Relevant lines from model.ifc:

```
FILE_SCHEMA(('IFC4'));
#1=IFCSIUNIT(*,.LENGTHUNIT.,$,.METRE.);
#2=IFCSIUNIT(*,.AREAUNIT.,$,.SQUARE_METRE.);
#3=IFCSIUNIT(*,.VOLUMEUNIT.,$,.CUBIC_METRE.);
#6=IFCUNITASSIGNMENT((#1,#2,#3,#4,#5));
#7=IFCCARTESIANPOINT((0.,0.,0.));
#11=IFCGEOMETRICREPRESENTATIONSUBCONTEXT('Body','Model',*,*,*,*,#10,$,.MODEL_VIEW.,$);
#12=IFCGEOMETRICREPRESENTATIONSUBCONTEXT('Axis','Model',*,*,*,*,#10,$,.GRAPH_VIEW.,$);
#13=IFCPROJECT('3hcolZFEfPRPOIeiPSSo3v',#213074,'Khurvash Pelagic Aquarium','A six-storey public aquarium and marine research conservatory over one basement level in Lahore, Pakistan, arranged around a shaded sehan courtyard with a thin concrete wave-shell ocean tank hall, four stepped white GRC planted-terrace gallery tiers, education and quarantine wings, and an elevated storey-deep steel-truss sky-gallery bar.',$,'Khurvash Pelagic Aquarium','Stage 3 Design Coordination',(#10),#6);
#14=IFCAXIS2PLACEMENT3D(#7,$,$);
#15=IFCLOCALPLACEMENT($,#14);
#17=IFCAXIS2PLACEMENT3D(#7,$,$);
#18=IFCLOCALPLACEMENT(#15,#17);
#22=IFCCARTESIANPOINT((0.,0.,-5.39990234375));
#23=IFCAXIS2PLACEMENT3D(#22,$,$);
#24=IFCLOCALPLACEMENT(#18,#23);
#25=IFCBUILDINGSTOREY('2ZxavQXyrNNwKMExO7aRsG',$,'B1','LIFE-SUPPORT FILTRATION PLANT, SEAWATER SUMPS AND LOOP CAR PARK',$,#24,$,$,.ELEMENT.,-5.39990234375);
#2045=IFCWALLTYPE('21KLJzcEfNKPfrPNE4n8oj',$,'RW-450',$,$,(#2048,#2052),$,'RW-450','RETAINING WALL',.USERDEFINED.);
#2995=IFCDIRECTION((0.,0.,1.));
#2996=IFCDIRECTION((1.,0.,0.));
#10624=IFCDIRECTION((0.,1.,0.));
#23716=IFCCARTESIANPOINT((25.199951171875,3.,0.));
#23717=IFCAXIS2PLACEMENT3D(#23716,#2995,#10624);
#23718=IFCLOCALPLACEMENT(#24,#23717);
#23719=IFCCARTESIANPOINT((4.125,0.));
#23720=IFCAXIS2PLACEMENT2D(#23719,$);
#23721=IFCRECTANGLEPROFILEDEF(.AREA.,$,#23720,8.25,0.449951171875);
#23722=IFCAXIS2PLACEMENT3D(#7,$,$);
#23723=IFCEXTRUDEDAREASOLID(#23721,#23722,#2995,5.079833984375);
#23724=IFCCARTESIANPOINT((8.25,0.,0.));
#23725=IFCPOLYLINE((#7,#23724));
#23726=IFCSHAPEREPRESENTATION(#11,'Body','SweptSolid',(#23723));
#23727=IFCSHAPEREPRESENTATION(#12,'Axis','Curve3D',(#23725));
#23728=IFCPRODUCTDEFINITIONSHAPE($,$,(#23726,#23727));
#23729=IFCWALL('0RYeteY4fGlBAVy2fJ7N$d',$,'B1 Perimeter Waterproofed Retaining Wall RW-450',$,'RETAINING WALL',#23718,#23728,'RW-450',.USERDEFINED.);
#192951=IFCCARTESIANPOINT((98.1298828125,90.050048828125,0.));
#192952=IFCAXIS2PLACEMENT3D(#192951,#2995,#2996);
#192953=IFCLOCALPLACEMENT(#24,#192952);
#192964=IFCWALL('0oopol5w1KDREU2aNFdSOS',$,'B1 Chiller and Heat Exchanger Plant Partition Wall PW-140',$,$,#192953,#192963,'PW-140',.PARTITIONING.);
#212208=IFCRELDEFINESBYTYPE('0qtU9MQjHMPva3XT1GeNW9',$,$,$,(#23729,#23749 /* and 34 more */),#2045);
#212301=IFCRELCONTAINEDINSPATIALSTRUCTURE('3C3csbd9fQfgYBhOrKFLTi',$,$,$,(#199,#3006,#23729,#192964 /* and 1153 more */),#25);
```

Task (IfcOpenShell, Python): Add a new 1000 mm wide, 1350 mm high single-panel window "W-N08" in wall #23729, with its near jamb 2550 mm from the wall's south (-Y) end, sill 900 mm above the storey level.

```python
import numpy as np
import ifcopenshell
import ifcopenshell.api.feature
import ifcopenshell.api.geometry
import ifcopenshell.api.root
import ifcopenshell.api.spatial
import ifcopenshell.geom
import ifcopenshell.util.element
import ifcopenshell.util.placement
import ifcopenshell.util.representation
import ifcopenshell.util.shape
import ifcopenshell.util.unit

model = ifcopenshell.open("model.ifc")
unit_scale = ifcopenshell.util.unit.calculate_unit_scale(model)
settings = ifcopenshell.geom.settings()


def volume(element):
    """Net volume in cubic metres, openings subtracted."""
    shape = ifcopenshell.geom.create_shape(settings, element)
    return ifcopenshell.util.shape.get_volume(shape.geometry)


wall = model.by_guid("0RYeteY4fGlBAVy2fJ7N$d")
storey = ifcopenshell.util.element.get_container(wall, ifc_class="IfcBuildingStorey")
context = ifcopenshell.util.representation.get_context(model, "Model", "Body", "MODEL_VIEW")
before = volume(wall)

width, height, from_end, sill = 1, 1.35, 2.55, 0.9  # metres

# The wall runs along its own X axis, and the end named is its -X end.
wall_shape = ifcopenshell.geom.create_shape(settings, wall)
x, y, z = ifcopenshell.util.shape.get_vertices(wall_shape.geometry).T
start = x.min() + from_end
face, thickness = float(y.min()), float(y.max() - y.min())
wall_matrix = ifcopenshell.util.placement.get_local_placement(wall.ObjectPlacement)
level = ifcopenshell.util.placement.get_local_placement(storey.ObjectPlacement)[2, 3]


def in_wall(x, y):
    """Placement at x, y metres in the wall's axes, at sill height."""
    matrix = wall_matrix.copy()
    matrix[:, 3] = wall_matrix @ np.array([x / unit_scale, y / unit_scale, 0.0, 1.0])
    matrix[2, 3] = level + sill / unit_scale
    return matrix


# Opening: a box that overshoots both wall faces by 50 mm.
opening = ifcopenshell.api.root.create_entity(model, ifc_class="IfcOpeningElement", predefined_type="OPENING")
box = ifcopenshell.api.geometry.add_wall_representation(
    model, context=context, length=width, height=height, thickness=thickness + 0.1
)
ifcopenshell.api.geometry.assign_representation(model, product=opening, representation=box)
ifcopenshell.api.geometry.edit_object_placement(model, product=opening, matrix=in_wall(start, face - 0.05), is_si=False)
ifcopenshell.api.feature.add_feature(model, feature=opening, element=wall)

window = ifcopenshell.api.root.create_entity(model, ifc_class="IfcWindow", name="W-N08", predefined_type="WINDOW")
window.OverallWidth, window.OverallHeight = width / unit_scale, height / unit_scale
window.PartitioningType = "SINGLE_PANEL"
body = ifcopenshell.api.geometry.add_window_representation(
    model,
    context=context,
    overall_width=window.OverallWidth,
    overall_height=window.OverallHeight,
    partition_type="SINGLE_PANEL",
)
ifcopenshell.api.geometry.assign_representation(model, product=window, representation=body)
ifcopenshell.api.spatial.assign_container(model, products=[window], relating_structure=storey)
ifcopenshell.api.feature.add_filling(model, opening=opening, element=window)

# Centre the window in the wall's thickness.
ifcopenshell.api.geometry.edit_object_placement(model, product=window, matrix=in_wall(start, face), is_si=False)
window_shape = ifcopenshell.geom.create_shape(settings, window)
depth = ifcopenshell.util.shape.get_vertices(window_shape.geometry)[:, 1]
offset = face + thickness / 2 - (depth.min() + depth.max()) / 2
ifcopenshell.api.geometry.edit_object_placement(model, product=window, matrix=in_wall(start, offset), is_si=False)

after = volume(wall)

print(f"wall volume {before:.3f} -> {after:.3f} m3")

model.write("model_edited.ifc")
```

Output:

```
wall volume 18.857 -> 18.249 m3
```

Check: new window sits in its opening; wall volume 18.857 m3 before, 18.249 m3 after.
